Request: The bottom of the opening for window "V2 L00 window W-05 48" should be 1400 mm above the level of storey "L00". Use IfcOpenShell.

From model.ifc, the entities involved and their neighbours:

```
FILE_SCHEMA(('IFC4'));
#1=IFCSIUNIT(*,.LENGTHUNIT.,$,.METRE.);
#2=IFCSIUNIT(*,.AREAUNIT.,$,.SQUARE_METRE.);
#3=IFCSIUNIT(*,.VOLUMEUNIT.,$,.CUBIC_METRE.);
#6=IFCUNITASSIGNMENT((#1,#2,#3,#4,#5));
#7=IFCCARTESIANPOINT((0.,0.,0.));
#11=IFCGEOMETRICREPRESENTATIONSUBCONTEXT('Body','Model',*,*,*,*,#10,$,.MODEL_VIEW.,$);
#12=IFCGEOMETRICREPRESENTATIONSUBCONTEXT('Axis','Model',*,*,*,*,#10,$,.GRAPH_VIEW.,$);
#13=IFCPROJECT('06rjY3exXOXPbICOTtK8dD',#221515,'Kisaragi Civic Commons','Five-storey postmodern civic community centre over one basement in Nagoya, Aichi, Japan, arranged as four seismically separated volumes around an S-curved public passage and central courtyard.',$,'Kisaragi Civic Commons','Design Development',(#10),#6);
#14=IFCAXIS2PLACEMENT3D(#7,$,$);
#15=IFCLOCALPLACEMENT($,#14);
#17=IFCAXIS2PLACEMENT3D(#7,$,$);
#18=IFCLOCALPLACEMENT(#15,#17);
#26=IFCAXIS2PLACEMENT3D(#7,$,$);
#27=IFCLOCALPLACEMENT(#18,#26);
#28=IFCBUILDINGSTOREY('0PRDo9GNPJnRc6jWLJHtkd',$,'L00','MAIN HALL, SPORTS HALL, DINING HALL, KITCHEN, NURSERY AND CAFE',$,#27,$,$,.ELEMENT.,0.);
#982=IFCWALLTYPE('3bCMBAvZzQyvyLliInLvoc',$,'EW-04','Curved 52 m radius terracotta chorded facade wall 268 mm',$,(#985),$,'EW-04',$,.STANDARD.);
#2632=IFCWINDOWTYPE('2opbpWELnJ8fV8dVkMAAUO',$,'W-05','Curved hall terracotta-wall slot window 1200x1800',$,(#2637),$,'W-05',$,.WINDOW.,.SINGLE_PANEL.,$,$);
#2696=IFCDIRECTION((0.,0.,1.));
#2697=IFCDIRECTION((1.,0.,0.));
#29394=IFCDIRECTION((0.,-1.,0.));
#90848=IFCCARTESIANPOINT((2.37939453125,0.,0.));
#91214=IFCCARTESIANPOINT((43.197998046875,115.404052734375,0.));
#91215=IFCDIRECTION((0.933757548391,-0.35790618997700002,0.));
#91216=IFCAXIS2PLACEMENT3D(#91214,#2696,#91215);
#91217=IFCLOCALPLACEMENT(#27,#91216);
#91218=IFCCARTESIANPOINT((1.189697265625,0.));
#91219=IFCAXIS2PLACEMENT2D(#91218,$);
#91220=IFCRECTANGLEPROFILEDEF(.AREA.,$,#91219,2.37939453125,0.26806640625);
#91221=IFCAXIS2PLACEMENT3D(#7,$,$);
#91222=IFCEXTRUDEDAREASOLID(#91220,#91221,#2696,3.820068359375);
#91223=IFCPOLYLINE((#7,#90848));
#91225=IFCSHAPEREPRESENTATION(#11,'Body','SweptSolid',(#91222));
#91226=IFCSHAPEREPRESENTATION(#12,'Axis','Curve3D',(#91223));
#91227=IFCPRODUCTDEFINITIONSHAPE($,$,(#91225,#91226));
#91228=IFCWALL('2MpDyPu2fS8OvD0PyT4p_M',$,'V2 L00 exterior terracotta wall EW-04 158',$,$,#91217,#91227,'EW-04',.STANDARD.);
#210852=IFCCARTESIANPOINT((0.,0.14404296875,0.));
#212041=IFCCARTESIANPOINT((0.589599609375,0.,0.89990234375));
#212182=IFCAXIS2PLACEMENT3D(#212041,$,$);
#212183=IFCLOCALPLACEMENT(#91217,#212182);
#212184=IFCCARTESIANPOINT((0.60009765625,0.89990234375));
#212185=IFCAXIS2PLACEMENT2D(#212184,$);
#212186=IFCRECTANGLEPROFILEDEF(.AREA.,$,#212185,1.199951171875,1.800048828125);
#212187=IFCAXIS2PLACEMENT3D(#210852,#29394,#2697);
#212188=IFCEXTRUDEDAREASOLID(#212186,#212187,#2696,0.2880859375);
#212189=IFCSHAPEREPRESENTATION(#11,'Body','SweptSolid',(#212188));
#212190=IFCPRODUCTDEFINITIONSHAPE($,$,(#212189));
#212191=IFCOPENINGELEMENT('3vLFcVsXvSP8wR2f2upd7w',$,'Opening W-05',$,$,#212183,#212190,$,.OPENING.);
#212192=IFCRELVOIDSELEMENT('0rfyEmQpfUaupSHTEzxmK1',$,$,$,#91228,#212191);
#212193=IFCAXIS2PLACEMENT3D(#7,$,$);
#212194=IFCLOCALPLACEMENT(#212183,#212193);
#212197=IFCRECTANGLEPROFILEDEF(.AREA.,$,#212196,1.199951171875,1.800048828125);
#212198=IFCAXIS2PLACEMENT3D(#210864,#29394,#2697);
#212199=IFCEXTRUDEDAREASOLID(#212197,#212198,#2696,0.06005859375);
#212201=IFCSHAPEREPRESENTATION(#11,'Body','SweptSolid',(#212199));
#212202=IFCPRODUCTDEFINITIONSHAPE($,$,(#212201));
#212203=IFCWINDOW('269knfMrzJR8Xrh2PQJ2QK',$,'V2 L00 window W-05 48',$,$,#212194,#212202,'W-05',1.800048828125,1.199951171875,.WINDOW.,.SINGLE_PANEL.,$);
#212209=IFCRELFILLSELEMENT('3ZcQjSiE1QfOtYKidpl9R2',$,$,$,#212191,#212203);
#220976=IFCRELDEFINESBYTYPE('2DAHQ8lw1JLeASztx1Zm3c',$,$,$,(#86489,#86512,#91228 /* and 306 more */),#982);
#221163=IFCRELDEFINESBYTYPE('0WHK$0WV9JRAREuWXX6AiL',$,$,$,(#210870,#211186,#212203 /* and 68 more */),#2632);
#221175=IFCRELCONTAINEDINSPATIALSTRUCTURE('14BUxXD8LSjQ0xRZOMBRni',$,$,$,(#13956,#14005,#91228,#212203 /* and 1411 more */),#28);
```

```python
import numpy as np
import ifcopenshell
import ifcopenshell.api.geometry
import ifcopenshell.geom
import ifcopenshell.util.element
import ifcopenshell.util.placement
import ifcopenshell.util.shape
import ifcopenshell.util.unit

model = ifcopenshell.open("model.ifc")
unit_scale = ifcopenshell.util.unit.calculate_unit_scale(model)

window = model.by_id(212203)
opening = window.FillsVoids[0].RelatingOpeningElement
storey = ifcopenshell.util.element.get_container(window, ifc_class="IfcBuildingStorey")
level = ifcopenshell.util.placement.get_local_placement(storey.ObjectPlacement)[2, 3]

# The opening's origin need not be at the sill, so measure its lowest point.
shape = ifcopenshell.geom.create_shape(ifcopenshell.geom.settings(), opening)
bottom = ifcopenshell.util.shape.get_shape_bottom_elevation(shape, shape.geometry) / unit_scale
dz = level + 1.4 - bottom

shift = np.array([0.0, 0.0, dz])
# The window is placed relative to its opening, so it follows when the opening moves.
matrix = ifcopenshell.util.placement.get_local_placement(opening.ObjectPlacement)
matrix[:3, 3] += shift
ifcopenshell.api.geometry.edit_object_placement(
    model, product=opening, matrix=matrix, is_si=False, should_transform_children=True
)

print(f"moved by {dz * unit_scale:+.3f} m")

model.write("model_updated.ifc")
```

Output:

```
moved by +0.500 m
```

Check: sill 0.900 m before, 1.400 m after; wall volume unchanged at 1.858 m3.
